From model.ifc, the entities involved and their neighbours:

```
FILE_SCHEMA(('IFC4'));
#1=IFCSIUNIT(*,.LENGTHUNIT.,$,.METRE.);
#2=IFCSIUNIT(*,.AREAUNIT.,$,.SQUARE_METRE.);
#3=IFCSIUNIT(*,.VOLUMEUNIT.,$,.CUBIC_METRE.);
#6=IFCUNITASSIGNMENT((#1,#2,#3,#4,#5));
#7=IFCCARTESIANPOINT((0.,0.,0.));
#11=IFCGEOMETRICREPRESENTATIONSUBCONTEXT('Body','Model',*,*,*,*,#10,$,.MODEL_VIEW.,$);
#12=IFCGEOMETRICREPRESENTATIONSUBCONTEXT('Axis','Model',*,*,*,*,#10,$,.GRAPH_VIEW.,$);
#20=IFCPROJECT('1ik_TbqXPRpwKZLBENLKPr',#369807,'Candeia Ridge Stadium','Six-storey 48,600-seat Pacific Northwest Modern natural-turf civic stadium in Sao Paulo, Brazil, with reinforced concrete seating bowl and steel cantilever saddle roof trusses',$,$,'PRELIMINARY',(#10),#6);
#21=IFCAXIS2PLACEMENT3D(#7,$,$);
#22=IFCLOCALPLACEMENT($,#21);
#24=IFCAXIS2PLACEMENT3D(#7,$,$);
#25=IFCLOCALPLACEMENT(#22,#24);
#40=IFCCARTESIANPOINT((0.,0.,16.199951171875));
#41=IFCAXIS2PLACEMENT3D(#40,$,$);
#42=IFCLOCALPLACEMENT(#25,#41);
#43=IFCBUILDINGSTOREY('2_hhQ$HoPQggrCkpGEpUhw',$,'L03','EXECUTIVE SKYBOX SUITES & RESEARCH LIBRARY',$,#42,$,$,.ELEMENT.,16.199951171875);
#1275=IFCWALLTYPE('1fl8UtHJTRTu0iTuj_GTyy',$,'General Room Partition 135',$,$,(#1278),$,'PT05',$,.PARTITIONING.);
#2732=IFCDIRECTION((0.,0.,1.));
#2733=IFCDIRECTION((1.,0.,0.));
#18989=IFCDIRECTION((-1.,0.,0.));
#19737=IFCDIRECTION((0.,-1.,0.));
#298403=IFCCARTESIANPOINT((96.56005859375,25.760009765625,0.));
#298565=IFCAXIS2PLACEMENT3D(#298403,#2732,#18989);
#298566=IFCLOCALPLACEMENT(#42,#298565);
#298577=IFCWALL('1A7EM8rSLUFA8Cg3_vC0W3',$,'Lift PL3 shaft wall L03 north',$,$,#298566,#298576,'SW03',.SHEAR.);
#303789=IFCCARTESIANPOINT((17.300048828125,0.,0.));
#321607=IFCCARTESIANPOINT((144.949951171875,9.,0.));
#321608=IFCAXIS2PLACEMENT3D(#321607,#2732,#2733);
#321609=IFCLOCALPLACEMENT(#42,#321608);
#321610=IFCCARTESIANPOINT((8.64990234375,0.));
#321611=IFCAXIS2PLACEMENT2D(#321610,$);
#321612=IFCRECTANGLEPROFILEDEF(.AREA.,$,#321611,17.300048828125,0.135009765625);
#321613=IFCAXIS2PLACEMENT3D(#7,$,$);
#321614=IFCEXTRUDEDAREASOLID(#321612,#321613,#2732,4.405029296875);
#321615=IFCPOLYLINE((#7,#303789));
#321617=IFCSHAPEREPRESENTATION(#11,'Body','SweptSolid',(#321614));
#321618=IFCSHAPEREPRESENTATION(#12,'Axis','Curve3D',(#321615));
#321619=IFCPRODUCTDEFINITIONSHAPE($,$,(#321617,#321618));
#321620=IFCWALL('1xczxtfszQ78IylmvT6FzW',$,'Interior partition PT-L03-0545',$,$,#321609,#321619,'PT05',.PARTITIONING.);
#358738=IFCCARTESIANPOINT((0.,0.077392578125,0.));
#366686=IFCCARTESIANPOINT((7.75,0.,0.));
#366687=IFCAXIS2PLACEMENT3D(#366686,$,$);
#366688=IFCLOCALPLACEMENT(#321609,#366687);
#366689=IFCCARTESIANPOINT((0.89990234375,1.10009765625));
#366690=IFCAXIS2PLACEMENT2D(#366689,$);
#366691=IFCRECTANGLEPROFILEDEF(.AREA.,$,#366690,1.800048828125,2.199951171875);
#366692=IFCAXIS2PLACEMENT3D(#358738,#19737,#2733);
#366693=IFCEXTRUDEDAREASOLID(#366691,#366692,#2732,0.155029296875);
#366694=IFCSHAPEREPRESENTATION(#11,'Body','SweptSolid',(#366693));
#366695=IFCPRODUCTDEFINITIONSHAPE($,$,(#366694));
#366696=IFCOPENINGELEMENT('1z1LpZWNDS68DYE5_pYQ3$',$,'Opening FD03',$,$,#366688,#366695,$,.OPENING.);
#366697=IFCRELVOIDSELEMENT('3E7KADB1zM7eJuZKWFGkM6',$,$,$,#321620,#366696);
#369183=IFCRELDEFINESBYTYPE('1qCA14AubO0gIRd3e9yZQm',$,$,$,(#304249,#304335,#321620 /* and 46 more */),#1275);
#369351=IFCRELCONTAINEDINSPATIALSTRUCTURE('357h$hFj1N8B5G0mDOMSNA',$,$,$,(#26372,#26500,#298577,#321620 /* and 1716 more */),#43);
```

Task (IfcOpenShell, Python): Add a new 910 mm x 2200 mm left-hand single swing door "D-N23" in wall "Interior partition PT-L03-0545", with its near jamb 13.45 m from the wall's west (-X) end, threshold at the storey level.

```python
import numpy as np
import ifcopenshell
import ifcopenshell.api.feature
import ifcopenshell.api.geometry
import ifcopenshell.api.root
import ifcopenshell.api.spatial
import ifcopenshell.geom
import ifcopenshell.util.element
import ifcopenshell.util.placement
import ifcopenshell.util.representation
import ifcopenshell.util.shape
import ifcopenshell.util.unit

model = ifcopenshell.open("model.ifc")
unit_scale = ifcopenshell.util.unit.calculate_unit_scale(model)
settings = ifcopenshell.geom.settings()


def volume(element):
    """Net volume in cubic metres, openings subtracted."""
    shape = ifcopenshell.geom.create_shape(settings, element)
    return ifcopenshell.util.shape.get_volume(shape.geometry)


wall = model.by_id(321620)
storey = ifcopenshell.util.element.get_container(wall, ifc_class="IfcBuildingStorey")
context = ifcopenshell.util.representation.get_context(model, "Model", "Body", "MODEL_VIEW")
before = volume(wall)

width, height, from_end, sill = 0.91, 2.2, 13.45, 0.0  # metres

# The wall runs along its own X axis, and the end named is its -X end.
wall_shape = ifcopenshell.geom.create_shape(settings, wall)
x, y, z = ifcopenshell.util.shape.get_vertices(wall_shape.geometry).T
start = x.min() + from_end
face, thickness = float(y.min()), float(y.max() - y.min())
wall_matrix = ifcopenshell.util.placement.get_local_placement(wall.ObjectPlacement)
level = ifcopenshell.util.placement.get_local_placement(storey.ObjectPlacement)[2, 3]


def in_wall(x, y):
    """Placement at x, y metres in the wall's axes, at sill height."""
    matrix = wall_matrix.copy()
    matrix[:, 3] = wall_matrix @ np.array([x / unit_scale, y / unit_scale, 0.0, 1.0])
    matrix[2, 3] = level + sill / unit_scale
    return matrix


# Opening: a box that overshoots both wall faces by 50 mm.
opening = ifcopenshell.api.root.create_entity(model, ifc_class="IfcOpeningElement", predefined_type="OPENING")
box = ifcopenshell.api.geometry.add_wall_representation(
    model, context=context, length=width, height=height, thickness=thickness + 0.1
)
ifcopenshell.api.geometry.assign_representation(model, product=opening, representation=box)
ifcopenshell.api.geometry.edit_object_placement(model, product=opening, matrix=in_wall(start, face - 0.05), is_si=False)
ifcopenshell.api.feature.add_feature(model, feature=opening, element=wall)

door = ifcopenshell.api.root.create_entity(model, ifc_class="IfcDoor", name="D-N23", predefined_type="DOOR")
door.OverallWidth, door.OverallHeight = width / unit_scale, height / unit_scale
door.OperationType = "SINGLE_SWING_LEFT"
body = ifcopenshell.api.geometry.add_door_representation(
    model,
    context=context,
    overall_width=door.OverallWidth,
    overall_height=door.OverallHeight,
    operation_type="SINGLE_SWING_LEFT",
    lining_properties={"LiningDepth": thickness / unit_scale, "ThresholdDepth": thickness / unit_scale},
)
ifcopenshell.api.geometry.assign_representation(model, product=door, representation=body)
ifcopenshell.api.spatial.assign_container(model, products=[door], relating_structure=storey)
ifcopenshell.api.feature.add_filling(model, opening=opening, element=door)

# The lining spans the wall, so the door starts at the wall face.
ifcopenshell.api.geometry.edit_object_placement(model, product=door, matrix=in_wall(start, face), is_si=False)

after = volume(wall)

print(f"wall volume {before:.3f} -> {after:.3f} m3")

model.write("model_v2.ifc")
```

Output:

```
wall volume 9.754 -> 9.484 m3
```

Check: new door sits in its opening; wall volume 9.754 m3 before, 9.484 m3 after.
